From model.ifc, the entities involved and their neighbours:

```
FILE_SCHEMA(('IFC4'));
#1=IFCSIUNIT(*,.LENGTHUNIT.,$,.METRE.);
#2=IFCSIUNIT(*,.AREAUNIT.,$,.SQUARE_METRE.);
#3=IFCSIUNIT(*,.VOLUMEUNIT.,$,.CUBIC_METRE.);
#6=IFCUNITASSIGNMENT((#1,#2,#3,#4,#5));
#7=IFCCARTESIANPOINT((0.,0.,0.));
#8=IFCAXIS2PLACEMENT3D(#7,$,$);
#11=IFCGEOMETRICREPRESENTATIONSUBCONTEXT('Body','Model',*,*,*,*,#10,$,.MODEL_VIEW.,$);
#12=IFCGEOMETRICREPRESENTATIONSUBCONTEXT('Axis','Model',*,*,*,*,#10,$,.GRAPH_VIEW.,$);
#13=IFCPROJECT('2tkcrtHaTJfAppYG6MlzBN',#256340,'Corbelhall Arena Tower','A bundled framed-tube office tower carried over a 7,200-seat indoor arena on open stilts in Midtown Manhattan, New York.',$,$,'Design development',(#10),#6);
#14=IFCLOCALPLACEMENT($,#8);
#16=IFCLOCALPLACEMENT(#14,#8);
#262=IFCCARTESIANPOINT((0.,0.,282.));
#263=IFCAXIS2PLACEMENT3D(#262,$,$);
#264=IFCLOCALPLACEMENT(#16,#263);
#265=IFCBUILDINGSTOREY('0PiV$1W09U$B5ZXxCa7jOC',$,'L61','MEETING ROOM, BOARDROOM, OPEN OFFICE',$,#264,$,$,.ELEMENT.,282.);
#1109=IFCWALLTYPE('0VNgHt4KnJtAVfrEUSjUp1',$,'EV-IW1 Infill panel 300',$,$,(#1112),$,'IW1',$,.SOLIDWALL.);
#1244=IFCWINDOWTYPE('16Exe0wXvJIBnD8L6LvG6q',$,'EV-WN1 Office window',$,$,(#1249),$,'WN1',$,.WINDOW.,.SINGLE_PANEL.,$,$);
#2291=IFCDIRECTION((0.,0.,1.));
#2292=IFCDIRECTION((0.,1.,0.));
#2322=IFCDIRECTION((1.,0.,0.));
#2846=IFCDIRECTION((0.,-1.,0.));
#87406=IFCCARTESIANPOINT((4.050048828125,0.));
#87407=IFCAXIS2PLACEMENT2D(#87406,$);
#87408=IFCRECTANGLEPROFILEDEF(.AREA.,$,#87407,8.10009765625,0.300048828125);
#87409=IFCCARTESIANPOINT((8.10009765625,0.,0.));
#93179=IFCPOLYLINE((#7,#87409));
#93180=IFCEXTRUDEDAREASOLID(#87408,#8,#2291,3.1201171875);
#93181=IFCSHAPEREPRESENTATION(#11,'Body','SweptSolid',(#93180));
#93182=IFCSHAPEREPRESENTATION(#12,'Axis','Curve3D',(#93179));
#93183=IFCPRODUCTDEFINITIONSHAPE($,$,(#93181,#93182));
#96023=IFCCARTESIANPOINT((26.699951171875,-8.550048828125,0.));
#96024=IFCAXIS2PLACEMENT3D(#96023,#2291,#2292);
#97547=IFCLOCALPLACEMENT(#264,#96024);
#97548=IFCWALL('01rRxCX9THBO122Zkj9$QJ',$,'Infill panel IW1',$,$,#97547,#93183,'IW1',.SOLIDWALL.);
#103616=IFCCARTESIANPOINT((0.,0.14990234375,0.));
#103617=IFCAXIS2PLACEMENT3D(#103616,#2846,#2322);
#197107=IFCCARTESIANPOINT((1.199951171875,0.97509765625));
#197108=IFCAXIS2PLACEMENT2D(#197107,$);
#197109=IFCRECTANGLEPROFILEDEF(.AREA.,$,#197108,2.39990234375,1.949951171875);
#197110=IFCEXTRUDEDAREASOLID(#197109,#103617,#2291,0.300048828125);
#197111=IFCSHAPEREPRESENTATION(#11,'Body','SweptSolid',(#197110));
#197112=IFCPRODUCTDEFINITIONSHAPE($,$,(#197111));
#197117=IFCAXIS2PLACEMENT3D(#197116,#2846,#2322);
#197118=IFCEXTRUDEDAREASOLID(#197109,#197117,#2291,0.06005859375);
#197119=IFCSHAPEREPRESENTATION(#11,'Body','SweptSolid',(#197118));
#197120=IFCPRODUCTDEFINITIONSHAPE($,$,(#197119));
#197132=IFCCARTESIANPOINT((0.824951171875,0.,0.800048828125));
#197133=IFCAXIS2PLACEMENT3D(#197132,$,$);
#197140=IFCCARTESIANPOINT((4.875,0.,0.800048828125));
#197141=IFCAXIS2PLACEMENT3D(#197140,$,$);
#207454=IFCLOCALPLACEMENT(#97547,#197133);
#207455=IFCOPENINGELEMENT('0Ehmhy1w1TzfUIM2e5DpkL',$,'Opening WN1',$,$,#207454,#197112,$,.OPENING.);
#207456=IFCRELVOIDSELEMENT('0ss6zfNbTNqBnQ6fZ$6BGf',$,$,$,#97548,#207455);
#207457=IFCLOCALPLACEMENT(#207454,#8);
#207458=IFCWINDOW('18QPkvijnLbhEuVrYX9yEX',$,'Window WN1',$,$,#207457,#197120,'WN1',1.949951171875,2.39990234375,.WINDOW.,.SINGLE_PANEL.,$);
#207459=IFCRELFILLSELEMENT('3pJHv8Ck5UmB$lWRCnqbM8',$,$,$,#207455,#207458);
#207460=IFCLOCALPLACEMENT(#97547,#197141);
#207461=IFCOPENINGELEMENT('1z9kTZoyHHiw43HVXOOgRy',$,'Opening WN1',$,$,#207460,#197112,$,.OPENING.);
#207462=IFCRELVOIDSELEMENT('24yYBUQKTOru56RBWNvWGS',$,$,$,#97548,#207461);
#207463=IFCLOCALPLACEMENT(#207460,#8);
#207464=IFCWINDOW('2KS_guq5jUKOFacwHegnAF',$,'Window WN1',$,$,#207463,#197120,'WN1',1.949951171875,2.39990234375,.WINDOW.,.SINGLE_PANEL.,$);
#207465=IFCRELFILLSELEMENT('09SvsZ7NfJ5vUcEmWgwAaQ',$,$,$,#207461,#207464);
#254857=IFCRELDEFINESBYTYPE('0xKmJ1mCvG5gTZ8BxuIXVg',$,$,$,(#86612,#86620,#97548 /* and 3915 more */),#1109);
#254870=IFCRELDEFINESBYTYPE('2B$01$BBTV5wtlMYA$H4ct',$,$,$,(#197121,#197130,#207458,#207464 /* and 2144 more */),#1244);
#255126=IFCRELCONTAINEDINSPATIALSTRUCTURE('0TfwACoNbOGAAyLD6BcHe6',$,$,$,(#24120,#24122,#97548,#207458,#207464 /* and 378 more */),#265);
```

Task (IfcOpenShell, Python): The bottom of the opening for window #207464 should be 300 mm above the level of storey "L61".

```python
import numpy as np
import ifcopenshell
import ifcopenshell.api.geometry
import ifcopenshell.geom
import ifcopenshell.util.element
import ifcopenshell.util.placement
import ifcopenshell.util.shape
import ifcopenshell.util.unit

model = ifcopenshell.open("model.ifc")
unit_scale = ifcopenshell.util.unit.calculate_unit_scale(model)

window = model.by_guid("2KS_guq5jUKOFacwHegnAF")
opening = window.FillsVoids[0].RelatingOpeningElement
storey = ifcopenshell.util.element.get_container(window, ifc_class="IfcBuildingStorey")
level = ifcopenshell.util.placement.get_local_placement(storey.ObjectPlacement)[2, 3]

# The opening's origin need not be at the sill, so measure its lowest point.
shape = ifcopenshell.geom.create_shape(ifcopenshell.geom.settings(), opening)
bottom = ifcopenshell.util.shape.get_shape_bottom_elevation(shape, shape.geometry) / unit_scale
dz = level + 0.3 / unit_scale - bottom

shift = np.array([0.0, 0.0, dz])
# The window is placed relative to its opening, so it follows when the opening moves.
matrix = ifcopenshell.util.placement.get_local_placement(opening.ObjectPlacement)
matrix[:3, 3] += shift
ifcopenshell.api.geometry.edit_object_placement(
    model, product=opening, matrix=matrix, is_si=False, should_transform_children=True
)

print(f"moved by {dz * unit_scale:+.3f} m")

model.write("model-out.ifc")
```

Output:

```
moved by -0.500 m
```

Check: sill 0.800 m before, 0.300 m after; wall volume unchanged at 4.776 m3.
